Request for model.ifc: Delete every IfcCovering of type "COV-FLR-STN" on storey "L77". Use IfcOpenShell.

First a look at what the model holds.

```python
import ifcopenshell
import ifcopenshell.util.element

model = ifcopenshell.open("model.ifc")
print(model.schema)
storey = next(s for s in model.by_type("IfcBuildingStorey") if s.Name == "L77")
coverings = [e for e in ifcopenshell.util.element.get_decomposition(storey) if e.is_a("IfcCovering")]
seen = {}
for e in coverings:
    element_type = ifcopenshell.util.element.get_type(e)
    name = element_type.Name if element_type not in (None, e) else None
    seen[name] = seen.get(name, 0) + 1
for name, count in sorted(seen.items(), key=str):
    print(count, "x", name)
```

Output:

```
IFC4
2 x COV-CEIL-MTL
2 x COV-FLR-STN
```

```python
import ifcopenshell
import ifcopenshell.api.root
import ifcopenshell.util.element

model = ifcopenshell.open("model.ifc")

storey = next(s for s in model.by_type("IfcBuildingStorey") if s.Name == "L77")
coverings = [e for e in ifcopenshell.util.element.get_decomposition(storey) if e.is_a("IfcCovering")]
targets = [e for e in coverings if (t := ifcopenshell.util.element.get_type(e)) not in (None, e) and t.Name == "COV-FLR-STN"]

for e in targets:
    ifcopenshell.api.root.remove_product(model, product=e)
print(len(targets), "removed")

model.write("model_edited.ifc")
```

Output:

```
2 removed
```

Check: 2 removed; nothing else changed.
